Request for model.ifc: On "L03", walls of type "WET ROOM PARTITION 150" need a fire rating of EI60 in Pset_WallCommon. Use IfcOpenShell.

First a look at what the model holds.

```python
import ifcopenshell
import ifcopenshell.util.element

model = ifcopenshell.open("model.ifc")
print(model.schema)
storey = next(s for s in model.by_type("IfcBuildingStorey") if s.Name == "L03")
walls = [e for e in ifcopenshell.util.element.get_decomposition(storey) if e.is_a("IfcWall")]
seen = {}
for e in walls:
    element_type = ifcopenshell.util.element.get_type(e)
    key = (element_type.Name if element_type != e and element_type else None, ifcopenshell.util.element.get_pset(e, "Pset_WallCommon", "FireRating"))
    seen[key] = seen.get(key, 0) + 1
for (name, value), count in sorted(seen.items(), key=str):
    print(count, "x", name, "|", value)
```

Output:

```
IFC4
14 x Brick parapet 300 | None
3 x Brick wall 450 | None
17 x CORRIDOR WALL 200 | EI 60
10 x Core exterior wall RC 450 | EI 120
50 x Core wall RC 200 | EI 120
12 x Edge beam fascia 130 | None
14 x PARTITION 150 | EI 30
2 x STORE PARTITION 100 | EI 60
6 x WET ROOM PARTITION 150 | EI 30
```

```python
import ifcopenshell
import ifcopenshell.api.pset
import ifcopenshell.util.element

model = ifcopenshell.open("model.ifc")

storey = next(s for s in model.by_type("IfcBuildingStorey") if s.Name == "L03")
walls = [e for e in ifcopenshell.util.element.get_decomposition(storey) if e.is_a("IfcWall")]

count = 0
for e in walls:
    element_type = ifcopenshell.util.element.get_type(e)
    if element_type in (None, e) or element_type.Name != "WET ROOM PARTITION 150":
        continue
    # add_pset returns the element's existing set when there is one.
    pset = ifcopenshell.api.pset.add_pset(model, product=e, name="Pset_WallCommon")
    ifcopenshell.api.pset.edit_pset(model, pset=pset, properties={"FireRating": "EI60"})
    count += 1

print(count, "walls updated")

model.write("model-out.ifc")
```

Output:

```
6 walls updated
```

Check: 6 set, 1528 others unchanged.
